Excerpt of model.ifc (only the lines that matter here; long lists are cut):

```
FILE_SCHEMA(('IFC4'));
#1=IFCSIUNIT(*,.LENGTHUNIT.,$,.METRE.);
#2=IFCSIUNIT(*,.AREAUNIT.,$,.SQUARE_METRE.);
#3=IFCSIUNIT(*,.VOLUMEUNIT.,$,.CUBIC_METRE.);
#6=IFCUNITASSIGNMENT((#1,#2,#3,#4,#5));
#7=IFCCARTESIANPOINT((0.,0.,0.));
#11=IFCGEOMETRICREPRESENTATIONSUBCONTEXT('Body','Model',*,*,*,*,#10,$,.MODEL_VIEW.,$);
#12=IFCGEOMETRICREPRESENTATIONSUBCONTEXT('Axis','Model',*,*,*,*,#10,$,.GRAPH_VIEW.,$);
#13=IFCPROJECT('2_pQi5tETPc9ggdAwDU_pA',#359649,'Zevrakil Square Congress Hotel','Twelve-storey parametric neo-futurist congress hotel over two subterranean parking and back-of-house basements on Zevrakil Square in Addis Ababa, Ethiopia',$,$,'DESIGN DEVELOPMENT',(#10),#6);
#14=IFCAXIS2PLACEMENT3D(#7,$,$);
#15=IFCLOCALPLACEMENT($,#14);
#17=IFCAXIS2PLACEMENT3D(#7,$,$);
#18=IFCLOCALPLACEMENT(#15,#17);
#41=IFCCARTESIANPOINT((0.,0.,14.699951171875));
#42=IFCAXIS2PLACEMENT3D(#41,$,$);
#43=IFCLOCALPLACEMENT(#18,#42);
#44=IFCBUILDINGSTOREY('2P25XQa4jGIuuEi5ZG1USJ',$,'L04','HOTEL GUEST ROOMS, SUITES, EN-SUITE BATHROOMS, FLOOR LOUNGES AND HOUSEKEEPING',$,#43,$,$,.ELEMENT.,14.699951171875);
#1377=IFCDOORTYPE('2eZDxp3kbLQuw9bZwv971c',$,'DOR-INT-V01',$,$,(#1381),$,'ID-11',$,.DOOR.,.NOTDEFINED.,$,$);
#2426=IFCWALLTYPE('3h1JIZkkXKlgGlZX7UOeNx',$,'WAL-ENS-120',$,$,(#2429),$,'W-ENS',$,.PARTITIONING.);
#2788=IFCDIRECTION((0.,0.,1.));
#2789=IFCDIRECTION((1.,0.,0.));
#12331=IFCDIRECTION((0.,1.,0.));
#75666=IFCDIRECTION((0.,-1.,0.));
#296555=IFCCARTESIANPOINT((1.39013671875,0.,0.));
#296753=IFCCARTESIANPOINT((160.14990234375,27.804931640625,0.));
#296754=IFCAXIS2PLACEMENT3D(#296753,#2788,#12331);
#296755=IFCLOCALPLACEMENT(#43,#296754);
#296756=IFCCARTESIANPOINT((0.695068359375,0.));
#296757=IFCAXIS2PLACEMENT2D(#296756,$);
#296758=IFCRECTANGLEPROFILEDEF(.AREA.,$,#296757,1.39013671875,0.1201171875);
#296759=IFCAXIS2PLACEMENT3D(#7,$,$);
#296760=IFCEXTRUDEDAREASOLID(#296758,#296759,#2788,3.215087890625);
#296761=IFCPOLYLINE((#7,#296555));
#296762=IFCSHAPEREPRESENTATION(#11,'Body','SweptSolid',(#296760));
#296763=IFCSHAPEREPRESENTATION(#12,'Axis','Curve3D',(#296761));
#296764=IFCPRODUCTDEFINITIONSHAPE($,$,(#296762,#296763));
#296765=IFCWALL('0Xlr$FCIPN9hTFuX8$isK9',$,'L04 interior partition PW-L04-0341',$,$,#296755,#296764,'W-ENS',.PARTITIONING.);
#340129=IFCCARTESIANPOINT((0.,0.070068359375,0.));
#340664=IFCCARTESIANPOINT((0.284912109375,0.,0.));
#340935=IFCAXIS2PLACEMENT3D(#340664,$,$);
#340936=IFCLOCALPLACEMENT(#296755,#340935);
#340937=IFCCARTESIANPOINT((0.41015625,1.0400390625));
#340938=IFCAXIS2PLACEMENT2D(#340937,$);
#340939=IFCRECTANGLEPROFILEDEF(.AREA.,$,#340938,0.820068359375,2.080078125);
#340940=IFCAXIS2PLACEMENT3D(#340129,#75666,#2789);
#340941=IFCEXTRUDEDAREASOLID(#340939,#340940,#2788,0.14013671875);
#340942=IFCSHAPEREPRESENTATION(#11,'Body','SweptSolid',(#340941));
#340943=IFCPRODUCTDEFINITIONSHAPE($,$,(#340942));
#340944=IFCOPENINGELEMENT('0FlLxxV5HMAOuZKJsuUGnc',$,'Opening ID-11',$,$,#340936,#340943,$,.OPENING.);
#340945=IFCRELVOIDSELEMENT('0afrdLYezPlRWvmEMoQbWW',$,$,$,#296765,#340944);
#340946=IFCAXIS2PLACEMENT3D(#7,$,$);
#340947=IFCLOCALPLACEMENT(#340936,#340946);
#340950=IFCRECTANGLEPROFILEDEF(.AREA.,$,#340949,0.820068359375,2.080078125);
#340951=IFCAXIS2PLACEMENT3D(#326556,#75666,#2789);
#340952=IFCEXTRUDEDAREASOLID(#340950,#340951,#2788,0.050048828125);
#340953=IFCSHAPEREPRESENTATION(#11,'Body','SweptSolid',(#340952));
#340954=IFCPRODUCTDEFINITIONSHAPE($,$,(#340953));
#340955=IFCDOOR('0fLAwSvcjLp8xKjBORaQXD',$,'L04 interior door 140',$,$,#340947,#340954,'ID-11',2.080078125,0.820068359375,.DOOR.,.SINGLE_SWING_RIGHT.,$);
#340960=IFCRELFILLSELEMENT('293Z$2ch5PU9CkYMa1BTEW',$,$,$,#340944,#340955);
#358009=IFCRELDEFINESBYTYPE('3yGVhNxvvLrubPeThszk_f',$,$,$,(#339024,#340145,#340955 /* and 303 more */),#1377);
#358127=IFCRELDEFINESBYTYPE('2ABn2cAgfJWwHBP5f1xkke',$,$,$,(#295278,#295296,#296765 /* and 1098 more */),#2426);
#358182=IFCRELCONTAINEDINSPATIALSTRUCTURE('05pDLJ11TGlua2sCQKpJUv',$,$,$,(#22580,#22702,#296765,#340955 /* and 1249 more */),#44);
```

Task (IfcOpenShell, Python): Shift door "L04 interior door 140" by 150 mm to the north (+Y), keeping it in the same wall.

```python
import ifcopenshell
import ifcopenshell.api.geometry
import ifcopenshell.util.placement
import ifcopenshell.util.unit

model = ifcopenshell.open("model.ifc")
unit_scale = ifcopenshell.util.unit.calculate_unit_scale(model)

door = model.by_guid("0fLAwSvcjLp8xKjBORaQXD")
opening = door.FillsVoids[0].RelatingOpeningElement
wall = opening.VoidsElements[0].RelatingBuildingElement

wall_matrix = ifcopenshell.util.placement.get_local_placement(wall.ObjectPlacement)
shift = wall_matrix[:3, 0] * 0.15 / unit_scale
before = ifcopenshell.util.placement.get_local_placement(door.ObjectPlacement)[:3, 3].copy()

# The door is placed relative to its opening, so it follows when the opening moves.
matrix = ifcopenshell.util.placement.get_local_placement(opening.ObjectPlacement)
matrix[:3, 3] += shift
ifcopenshell.api.geometry.edit_object_placement(
    model, product=opening, matrix=matrix, is_si=False, should_transform_children=True
)

after = ifcopenshell.util.placement.get_local_placement(door.ObjectPlacement)[:3, 3]
print("door moved by", (after - before).round(3) + 0.0)

model.write("model-out.ifc")
```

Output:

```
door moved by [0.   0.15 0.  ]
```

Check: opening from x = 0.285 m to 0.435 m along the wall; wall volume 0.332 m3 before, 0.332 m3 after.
